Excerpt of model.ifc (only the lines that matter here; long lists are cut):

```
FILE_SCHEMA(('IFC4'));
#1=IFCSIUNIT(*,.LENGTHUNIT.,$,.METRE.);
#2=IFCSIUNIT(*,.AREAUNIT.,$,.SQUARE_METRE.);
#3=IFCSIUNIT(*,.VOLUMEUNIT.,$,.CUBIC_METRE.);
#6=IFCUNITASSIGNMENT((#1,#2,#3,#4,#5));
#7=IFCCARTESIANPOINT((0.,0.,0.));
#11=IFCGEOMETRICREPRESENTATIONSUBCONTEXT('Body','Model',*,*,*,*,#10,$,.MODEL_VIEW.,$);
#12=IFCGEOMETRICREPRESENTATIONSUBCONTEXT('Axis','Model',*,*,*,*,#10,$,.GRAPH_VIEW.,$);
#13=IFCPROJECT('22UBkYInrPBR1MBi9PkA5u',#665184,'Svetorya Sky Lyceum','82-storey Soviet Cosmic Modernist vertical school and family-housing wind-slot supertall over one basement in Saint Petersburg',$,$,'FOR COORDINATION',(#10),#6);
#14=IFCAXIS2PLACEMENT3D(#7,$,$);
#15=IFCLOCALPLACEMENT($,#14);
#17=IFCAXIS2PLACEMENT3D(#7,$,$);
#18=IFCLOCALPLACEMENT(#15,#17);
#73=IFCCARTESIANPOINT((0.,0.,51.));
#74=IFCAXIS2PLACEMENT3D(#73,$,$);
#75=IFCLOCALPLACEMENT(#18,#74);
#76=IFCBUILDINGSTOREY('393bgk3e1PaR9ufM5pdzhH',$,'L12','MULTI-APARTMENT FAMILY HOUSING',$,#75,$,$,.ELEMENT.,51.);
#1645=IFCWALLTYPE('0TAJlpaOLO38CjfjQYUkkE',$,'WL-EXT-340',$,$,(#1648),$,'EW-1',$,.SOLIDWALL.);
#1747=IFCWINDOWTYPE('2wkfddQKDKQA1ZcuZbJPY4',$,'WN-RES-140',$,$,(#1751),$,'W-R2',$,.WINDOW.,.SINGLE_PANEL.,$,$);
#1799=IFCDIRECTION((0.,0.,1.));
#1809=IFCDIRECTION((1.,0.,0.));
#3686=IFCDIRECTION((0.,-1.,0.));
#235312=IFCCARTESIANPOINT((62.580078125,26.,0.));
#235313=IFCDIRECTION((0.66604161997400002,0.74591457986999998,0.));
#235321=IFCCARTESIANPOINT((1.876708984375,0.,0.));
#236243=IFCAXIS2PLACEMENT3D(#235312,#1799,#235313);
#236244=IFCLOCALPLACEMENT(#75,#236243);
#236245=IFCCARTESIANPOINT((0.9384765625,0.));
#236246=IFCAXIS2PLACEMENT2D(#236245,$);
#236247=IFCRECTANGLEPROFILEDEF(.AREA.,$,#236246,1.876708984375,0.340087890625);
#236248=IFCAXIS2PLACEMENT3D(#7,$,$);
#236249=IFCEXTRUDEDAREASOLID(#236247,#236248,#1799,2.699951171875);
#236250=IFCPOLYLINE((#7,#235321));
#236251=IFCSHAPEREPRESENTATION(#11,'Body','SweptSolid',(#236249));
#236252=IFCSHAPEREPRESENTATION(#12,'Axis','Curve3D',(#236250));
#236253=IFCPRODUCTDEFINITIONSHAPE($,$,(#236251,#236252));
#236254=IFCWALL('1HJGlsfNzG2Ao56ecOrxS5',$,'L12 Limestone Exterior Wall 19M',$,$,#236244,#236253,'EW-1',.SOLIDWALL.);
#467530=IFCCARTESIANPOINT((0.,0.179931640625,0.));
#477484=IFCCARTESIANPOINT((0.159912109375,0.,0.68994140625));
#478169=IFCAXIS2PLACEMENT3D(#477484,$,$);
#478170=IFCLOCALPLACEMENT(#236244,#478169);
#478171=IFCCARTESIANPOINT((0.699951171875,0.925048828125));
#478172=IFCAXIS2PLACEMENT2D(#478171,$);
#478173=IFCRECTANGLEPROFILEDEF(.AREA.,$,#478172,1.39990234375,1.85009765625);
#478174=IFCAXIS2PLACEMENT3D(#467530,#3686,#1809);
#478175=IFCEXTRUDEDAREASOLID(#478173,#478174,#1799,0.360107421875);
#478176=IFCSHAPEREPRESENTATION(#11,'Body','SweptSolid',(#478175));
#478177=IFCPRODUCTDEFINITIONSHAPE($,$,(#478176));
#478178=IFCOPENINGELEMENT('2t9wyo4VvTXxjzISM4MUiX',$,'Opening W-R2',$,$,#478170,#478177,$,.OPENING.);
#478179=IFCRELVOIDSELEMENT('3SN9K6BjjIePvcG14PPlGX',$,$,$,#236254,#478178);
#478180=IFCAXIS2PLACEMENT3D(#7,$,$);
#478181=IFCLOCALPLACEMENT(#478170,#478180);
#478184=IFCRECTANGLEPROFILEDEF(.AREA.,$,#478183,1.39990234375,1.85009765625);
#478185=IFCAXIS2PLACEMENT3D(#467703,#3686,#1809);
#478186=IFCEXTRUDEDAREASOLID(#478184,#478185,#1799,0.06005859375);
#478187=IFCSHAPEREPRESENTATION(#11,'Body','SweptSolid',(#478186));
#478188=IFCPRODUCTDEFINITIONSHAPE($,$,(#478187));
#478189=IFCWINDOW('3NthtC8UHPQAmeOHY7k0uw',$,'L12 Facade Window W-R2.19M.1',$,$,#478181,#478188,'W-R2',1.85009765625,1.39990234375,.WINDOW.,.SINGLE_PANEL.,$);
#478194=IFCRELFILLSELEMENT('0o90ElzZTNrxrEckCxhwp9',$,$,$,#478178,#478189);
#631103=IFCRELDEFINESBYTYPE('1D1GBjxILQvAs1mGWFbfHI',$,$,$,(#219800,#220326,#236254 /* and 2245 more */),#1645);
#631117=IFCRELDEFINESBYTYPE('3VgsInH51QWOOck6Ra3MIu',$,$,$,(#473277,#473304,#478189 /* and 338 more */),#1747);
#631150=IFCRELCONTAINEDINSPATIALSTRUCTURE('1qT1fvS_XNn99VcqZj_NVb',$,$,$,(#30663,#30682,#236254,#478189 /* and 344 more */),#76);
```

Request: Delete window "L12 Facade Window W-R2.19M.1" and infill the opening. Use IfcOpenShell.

```python
import ifcopenshell
import ifcopenshell.api.feature
import ifcopenshell.api.root
import ifcopenshell.geom
import ifcopenshell.util.shape

model = ifcopenshell.open("model.ifc")
settings = ifcopenshell.geom.settings()


def volume(element):
    """Net volume in cubic metres, openings subtracted."""
    shape = ifcopenshell.geom.create_shape(settings, element)
    return ifcopenshell.util.shape.get_volume(shape.geometry)


window = model.by_guid("3NthtC8UHPQAmeOHY7k0uw")
opening = window.FillsVoids[0].RelatingOpeningElement
wall = opening.VoidsElements[0].RelatingBuildingElement
before = volume(wall)

ifcopenshell.api.root.remove_product(model, product=window)
ifcopenshell.api.feature.remove_feature(model, feature=opening)

after = volume(wall)

print(f"wall volume {before:.3f} -> {after:.3f} m3")

model.write("model_v2.ifc")
```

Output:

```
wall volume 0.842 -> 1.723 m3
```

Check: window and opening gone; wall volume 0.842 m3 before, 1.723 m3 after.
